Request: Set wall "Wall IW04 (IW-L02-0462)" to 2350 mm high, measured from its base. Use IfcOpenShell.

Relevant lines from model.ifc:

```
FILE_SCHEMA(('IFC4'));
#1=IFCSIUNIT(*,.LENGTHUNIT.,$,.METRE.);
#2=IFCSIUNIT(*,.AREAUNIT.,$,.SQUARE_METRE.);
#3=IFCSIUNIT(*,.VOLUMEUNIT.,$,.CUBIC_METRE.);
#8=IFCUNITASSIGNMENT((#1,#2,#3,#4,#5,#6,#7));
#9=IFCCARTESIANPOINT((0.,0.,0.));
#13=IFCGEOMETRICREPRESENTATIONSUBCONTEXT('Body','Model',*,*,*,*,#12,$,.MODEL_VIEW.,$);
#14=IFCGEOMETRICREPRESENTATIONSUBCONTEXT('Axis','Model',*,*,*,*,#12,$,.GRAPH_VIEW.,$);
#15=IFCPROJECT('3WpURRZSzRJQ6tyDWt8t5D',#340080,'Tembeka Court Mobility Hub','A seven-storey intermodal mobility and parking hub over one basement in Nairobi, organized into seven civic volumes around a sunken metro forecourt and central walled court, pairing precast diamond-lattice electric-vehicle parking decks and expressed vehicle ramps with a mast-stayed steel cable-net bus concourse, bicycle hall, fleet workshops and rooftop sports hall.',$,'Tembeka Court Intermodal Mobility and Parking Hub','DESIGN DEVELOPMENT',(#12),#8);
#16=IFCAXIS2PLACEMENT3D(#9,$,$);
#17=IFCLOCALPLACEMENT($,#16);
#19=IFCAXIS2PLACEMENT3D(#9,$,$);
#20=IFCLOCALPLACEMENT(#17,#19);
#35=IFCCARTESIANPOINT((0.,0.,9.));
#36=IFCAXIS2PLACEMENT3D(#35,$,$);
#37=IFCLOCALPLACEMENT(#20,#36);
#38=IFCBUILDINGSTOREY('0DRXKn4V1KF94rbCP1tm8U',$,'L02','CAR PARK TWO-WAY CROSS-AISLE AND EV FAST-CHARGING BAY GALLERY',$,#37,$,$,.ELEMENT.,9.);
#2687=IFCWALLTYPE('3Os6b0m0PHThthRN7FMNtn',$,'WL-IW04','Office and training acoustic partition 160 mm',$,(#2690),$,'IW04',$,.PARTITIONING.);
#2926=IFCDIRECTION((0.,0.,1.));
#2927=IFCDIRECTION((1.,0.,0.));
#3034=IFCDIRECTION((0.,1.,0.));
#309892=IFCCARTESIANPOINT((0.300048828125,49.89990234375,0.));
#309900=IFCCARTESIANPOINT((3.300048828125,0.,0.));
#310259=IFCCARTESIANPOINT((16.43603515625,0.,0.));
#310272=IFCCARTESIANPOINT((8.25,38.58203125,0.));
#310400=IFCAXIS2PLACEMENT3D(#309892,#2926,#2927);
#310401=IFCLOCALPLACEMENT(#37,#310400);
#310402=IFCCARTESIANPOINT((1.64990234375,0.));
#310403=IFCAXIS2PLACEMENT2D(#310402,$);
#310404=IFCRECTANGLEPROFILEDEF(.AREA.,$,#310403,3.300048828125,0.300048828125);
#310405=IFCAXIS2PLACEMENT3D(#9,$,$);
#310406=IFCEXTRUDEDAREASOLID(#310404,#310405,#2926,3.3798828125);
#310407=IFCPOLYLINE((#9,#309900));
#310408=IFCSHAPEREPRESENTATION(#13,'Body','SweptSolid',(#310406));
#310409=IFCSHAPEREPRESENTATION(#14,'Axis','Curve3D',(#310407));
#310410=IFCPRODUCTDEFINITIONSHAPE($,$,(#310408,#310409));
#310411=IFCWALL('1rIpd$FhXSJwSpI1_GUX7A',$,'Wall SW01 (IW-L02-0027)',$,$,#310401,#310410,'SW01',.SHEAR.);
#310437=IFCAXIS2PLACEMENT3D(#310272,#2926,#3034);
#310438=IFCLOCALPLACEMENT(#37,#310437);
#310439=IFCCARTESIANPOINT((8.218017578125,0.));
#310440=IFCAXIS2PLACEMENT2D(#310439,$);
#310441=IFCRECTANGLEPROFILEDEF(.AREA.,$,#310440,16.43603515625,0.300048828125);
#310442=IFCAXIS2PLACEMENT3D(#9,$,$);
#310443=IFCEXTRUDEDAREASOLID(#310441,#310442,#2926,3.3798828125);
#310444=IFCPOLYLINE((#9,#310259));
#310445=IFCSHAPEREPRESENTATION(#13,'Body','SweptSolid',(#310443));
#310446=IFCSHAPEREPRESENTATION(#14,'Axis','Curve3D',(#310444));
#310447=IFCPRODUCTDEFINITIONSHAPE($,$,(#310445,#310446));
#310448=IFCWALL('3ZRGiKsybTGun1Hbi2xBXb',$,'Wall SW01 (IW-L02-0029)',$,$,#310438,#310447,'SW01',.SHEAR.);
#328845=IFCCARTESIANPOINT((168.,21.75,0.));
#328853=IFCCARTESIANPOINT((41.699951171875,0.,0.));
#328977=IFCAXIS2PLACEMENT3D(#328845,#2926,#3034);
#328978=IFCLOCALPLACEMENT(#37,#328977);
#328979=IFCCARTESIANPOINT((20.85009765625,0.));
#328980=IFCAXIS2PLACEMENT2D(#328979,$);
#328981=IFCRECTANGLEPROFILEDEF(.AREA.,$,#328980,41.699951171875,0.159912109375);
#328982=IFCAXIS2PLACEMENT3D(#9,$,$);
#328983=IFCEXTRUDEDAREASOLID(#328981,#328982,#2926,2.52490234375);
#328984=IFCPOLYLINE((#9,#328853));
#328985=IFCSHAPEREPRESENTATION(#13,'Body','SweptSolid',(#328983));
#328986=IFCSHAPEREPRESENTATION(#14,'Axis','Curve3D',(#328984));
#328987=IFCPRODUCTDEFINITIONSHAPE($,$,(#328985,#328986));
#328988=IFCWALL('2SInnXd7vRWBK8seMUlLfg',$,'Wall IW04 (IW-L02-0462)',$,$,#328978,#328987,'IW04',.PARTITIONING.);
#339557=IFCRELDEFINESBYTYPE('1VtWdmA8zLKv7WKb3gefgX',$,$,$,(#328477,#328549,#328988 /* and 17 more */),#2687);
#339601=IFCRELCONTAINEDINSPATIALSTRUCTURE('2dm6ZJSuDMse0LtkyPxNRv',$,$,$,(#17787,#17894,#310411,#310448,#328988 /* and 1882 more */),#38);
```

```python
import ifcopenshell
import ifcopenshell.geom
import ifcopenshell.util.representation
import ifcopenshell.util.shape

model = ifcopenshell.open("model.ifc")
settings = ifcopenshell.geom.settings()


def volume(element):
    """Net volume in cubic metres, openings subtracted."""
    shape = ifcopenshell.geom.create_shape(settings, element)
    return ifcopenshell.util.shape.get_volume(shape.geometry)


wall = model.by_guid("2SInnXd7vRWBK8seMUlLfg")
before = volume(wall)

body = ifcopenshell.util.representation.get_representation(wall, "Model", "Body")
solid = body.Items[0]
old_height = solid.Depth
solid.Depth = 2.35
after = volume(wall)

print(f"height {old_height:g} -> {solid.Depth:g}, volume {before:.3f} -> {after:.3f} m3")

model.write("model_v2.ifc")
```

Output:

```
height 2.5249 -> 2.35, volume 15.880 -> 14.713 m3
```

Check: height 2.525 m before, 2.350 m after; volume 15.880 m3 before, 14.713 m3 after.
